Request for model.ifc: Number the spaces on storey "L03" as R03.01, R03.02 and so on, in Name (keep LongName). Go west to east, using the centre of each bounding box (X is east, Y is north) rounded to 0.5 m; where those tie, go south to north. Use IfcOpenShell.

First a look at what the model holds.

```python
import ifcopenshell
import ifcopenshell.util.element
import ifcopenshell.util.placement

model = ifcopenshell.open("model.ifc")
print(model.schema)
storey = next(s for s in model.by_type("IfcBuildingStorey") if s.Name == "L03")
spaces = [e for e in ifcopenshell.util.element.get_decomposition(storey) if e.is_a("IfcSpace")]
for e in sorted(spaces, key=lambda e: e.id()):
    origin = ifcopenshell.util.placement.get_local_placement(e.ObjectPlacement)[:3, 3]
    print(e.id(), e.Name, e.LongName, origin.round(2) + 0.0, sep=" | ")
```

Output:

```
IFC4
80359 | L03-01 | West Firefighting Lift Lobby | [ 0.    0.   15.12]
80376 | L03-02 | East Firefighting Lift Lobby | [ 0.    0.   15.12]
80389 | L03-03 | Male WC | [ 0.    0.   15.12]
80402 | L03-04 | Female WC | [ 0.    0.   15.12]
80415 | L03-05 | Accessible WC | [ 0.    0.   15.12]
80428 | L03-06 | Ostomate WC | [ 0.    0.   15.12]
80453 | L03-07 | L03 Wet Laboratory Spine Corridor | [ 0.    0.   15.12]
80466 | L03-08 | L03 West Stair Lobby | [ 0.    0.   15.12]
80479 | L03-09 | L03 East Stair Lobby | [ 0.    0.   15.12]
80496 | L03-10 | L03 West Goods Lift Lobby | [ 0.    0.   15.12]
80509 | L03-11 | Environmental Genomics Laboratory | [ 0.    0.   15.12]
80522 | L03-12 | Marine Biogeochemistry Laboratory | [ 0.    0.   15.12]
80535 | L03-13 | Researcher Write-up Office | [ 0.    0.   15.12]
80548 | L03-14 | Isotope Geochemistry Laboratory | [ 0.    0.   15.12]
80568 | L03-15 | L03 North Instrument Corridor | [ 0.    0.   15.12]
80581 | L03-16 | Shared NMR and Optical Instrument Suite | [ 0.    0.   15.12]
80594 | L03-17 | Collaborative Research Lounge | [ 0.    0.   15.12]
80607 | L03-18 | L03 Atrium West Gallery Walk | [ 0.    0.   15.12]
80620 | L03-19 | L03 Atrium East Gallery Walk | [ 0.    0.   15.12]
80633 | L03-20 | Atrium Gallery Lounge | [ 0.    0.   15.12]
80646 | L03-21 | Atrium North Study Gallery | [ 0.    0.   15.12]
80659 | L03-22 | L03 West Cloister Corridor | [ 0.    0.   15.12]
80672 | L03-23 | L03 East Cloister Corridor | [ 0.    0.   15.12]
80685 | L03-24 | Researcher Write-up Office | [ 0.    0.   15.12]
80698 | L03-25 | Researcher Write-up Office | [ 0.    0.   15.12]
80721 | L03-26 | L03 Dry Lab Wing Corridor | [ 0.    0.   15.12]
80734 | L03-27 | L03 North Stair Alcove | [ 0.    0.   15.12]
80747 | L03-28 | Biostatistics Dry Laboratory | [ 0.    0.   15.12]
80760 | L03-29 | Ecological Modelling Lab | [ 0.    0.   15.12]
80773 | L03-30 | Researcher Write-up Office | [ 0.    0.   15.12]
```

```python
import ifcopenshell
import ifcopenshell.geom
import ifcopenshell.util.element
import ifcopenshell.util.shape

model = ifcopenshell.open("model.ifc")
settings = ifcopenshell.geom.settings()
settings.set("use-world-coords", True)


def centre(element):
    shape = ifcopenshell.geom.create_shape(settings, element)
    return ifcopenshell.util.shape.get_bbox_centroid(shape.geometry)


storey = next(s for s in model.by_type("IfcBuildingStorey") if s.Name == "L03")
spaces = [e for e in ifcopenshell.util.element.get_decomposition(storey) if e.is_a("IfcSpace")]

# Insertion points can sit at a corner or the storey origin, so sort by the geometry (in metres).
centres = {e: centre(e) for e in spaces}
spaces.sort(key=lambda e: (round(centres[e][0] / 0.5), centres[e][1]))

for i, e in enumerate(spaces, start=1):
    number = f"R03.{i:02d}"
    e.Name = number
    print(e.id(), number)

model.write("model_edited.ifc")
```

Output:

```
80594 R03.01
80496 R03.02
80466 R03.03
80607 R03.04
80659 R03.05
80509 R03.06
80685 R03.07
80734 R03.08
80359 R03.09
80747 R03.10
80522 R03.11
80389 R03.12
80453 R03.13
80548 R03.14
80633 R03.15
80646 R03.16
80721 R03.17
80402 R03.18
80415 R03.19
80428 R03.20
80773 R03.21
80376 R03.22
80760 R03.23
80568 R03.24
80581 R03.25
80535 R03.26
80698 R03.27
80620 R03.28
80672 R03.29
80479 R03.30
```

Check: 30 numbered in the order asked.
